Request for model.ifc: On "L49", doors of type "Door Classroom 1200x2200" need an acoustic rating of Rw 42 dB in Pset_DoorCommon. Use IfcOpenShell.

First a look at what the model holds.

```python
import ifcopenshell
import ifcopenshell.util.element

model = ifcopenshell.open("model.ifc")
print(model.schema)
storey = next(s for s in model.by_type("IfcBuildingStorey") if s.Name == "L49")
doors = [e for e in ifcopenshell.util.element.get_decomposition(storey) if e.is_a("IfcDoor")]
seen = {}
for e in doors:
    element_type = ifcopenshell.util.element.get_type(e)
    key = (element_type.Name if element_type != e and element_type else None, ifcopenshell.util.element.get_pset(e, "Pset_DoorCommon", "AcousticRating"))
    seen[key] = seen.get(key, 0) + 1
for (name, value), count in sorted(seen.items(), key=str):
    print(count, "x", name, "|", value)
```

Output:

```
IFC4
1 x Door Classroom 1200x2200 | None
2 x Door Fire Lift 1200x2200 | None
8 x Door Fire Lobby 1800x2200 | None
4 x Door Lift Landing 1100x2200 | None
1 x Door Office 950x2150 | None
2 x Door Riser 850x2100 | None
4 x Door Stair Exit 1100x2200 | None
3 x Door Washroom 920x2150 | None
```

```python
import ifcopenshell
import ifcopenshell.api.pset
import ifcopenshell.util.element

model = ifcopenshell.open("model.ifc")

storey = next(s for s in model.by_type("IfcBuildingStorey") if s.Name == "L49")
doors = [e for e in ifcopenshell.util.element.get_decomposition(storey) if e.is_a("IfcDoor")]

count = 0
for e in doors:
    element_type = ifcopenshell.util.element.get_type(e)
    if element_type in (None, e) or element_type.Name != "Door Classroom 1200x2200":
        continue
    found = ifcopenshell.util.element.get_pset(e, "Pset_DoorCommon", should_inherit=False)
    if found:
        pset = model.by_id(found["id"])
        if len(ifcopenshell.util.element.get_elements_by_pset(pset)) > 1:
            pset = ifcopenshell.api.pset.unshare_pset(model, products=[e], pset=pset)[0]
    else:
        pset = ifcopenshell.api.pset.add_pset(model, product=e, name="Pset_DoorCommon")
    ifcopenshell.api.pset.edit_pset(model, pset=pset, properties={"AcousticRating": "Rw 42 dB"})
    count += 1

print(count, "doors updated")

model.write("model_edited.ifc")
```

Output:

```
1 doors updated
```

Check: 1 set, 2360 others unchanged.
